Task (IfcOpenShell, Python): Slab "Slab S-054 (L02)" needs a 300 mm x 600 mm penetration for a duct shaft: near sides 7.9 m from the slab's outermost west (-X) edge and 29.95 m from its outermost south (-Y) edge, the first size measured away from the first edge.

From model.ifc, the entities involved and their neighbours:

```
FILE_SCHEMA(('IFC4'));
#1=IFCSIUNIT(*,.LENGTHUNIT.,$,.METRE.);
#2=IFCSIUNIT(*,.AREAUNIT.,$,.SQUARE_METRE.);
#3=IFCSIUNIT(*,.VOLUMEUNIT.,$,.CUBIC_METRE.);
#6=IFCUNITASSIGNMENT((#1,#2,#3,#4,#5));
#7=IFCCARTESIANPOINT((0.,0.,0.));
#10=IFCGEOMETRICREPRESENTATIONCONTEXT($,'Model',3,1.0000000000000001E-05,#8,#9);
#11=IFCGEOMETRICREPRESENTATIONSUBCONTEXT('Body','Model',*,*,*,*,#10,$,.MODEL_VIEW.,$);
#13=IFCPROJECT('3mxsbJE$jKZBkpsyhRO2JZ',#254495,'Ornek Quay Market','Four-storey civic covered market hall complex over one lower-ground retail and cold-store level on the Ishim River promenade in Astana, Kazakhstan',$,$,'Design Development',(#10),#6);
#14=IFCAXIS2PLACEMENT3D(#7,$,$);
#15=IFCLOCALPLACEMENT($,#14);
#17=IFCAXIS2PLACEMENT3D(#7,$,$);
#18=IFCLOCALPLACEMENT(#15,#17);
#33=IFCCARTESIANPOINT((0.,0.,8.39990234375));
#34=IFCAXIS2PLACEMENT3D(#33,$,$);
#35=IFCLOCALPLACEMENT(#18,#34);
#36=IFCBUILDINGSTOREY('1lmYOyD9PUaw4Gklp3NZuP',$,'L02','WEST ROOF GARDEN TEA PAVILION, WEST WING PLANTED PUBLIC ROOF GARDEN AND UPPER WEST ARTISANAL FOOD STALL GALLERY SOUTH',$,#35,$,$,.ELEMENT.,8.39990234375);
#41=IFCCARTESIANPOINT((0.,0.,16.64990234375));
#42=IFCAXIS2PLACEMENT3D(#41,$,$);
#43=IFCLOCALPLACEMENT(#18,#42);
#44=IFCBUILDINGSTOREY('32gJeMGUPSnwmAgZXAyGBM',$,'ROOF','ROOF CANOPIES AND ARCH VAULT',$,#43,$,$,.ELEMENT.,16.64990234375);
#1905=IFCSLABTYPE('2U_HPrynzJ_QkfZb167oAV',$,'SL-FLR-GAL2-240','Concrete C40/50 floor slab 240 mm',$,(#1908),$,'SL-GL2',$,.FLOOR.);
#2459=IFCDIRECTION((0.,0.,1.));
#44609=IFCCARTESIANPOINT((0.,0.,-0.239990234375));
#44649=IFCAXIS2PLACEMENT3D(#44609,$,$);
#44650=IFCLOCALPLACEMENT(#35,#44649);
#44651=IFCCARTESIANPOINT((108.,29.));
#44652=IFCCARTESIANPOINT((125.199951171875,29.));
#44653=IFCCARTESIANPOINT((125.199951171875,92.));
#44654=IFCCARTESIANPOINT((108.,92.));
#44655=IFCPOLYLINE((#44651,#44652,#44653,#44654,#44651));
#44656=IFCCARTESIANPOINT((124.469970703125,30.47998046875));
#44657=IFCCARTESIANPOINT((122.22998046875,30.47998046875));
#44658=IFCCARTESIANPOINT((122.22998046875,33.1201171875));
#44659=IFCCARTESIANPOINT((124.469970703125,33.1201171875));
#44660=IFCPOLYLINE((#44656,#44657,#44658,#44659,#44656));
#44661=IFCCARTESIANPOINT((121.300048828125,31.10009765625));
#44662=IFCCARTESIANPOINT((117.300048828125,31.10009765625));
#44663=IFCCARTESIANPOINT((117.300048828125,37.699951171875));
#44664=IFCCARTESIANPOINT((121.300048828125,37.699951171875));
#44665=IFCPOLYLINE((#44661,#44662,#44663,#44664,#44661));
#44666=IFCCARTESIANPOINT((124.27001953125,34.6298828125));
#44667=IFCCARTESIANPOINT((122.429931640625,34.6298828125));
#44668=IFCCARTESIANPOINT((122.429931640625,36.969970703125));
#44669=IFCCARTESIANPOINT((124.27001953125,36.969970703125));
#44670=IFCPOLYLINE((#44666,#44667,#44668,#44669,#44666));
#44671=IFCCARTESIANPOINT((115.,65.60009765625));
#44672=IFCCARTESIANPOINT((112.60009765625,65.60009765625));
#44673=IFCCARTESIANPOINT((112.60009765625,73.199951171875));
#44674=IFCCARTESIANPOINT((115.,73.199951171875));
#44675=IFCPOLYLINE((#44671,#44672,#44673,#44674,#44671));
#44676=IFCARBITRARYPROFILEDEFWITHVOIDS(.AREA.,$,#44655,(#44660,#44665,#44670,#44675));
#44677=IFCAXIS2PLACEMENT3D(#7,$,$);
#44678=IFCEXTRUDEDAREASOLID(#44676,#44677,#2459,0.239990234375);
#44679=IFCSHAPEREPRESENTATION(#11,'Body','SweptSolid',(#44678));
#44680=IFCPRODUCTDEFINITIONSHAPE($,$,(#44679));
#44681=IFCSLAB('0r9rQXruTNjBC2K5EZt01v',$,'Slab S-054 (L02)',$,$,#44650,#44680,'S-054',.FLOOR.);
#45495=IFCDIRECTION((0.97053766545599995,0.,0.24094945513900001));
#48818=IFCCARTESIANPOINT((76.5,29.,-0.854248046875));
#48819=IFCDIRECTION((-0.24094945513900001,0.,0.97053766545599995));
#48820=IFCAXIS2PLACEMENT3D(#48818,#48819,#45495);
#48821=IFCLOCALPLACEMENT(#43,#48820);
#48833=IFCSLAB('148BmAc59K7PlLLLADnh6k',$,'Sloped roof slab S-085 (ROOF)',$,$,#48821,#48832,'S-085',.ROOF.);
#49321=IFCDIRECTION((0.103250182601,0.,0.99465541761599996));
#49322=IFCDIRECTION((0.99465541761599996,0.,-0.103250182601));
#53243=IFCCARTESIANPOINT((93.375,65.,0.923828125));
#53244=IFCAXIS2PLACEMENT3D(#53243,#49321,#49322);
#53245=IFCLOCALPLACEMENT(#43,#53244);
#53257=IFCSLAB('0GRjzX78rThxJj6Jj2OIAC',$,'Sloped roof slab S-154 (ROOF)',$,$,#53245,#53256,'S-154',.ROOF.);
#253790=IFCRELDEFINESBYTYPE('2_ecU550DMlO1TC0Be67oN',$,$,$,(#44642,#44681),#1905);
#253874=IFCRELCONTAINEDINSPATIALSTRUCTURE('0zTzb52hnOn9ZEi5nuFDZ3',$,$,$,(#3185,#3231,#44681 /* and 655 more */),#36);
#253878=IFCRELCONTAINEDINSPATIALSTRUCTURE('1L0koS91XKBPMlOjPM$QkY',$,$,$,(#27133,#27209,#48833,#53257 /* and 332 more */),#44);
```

```python
import numpy as np
import ifcopenshell
import ifcopenshell.api.feature
import ifcopenshell.api.geometry
import ifcopenshell.api.root
import ifcopenshell.geom
import ifcopenshell.util.placement
import ifcopenshell.util.representation
import ifcopenshell.util.shape
import ifcopenshell.util.unit

model = ifcopenshell.open("model.ifc")
unit_scale = ifcopenshell.util.unit.calculate_unit_scale(model)
settings = ifcopenshell.geom.settings()


def volume(element):
    """Net volume in cubic metres, openings subtracted."""
    shape = ifcopenshell.geom.create_shape(settings, element)
    return ifcopenshell.util.shape.get_volume(shape.geometry)


slab = model.by_guid("0r9rQXruTNjBC2K5EZt01v")
before = volume(slab)

# Extent in the slab's own axes, in metres. The edges named are its -X and -Y sides.
slab_shape = ifcopenshell.geom.create_shape(settings, slab)
vertices = ifcopenshell.util.shape.get_vertices(slab_shape.geometry)
x_min, y_min, bottom = vertices.min(axis=0)
top = vertices[:, 2].max()

opening = ifcopenshell.api.root.create_entity(model, ifc_class="IfcOpeningElement", name="Duct shaft opening", predefined_type="OPENING")
context = ifcopenshell.util.representation.get_context(model, "Model", "Body", "MODEL_VIEW")
width, depth = 0.3, 0.6
outline = [(0.0, 0.0), (width, 0.0), (width, depth), (0.0, depth), (0.0, 0.0)]
# Overshoot both faces by 50 mm so the cut is clean.
shape = ifcopenshell.api.geometry.add_slab_representation(
    model, context=context, depth=top - bottom + 0.1, polyline=outline
)
ifcopenshell.api.geometry.assign_representation(model, product=opening, representation=shape)

matrix = ifcopenshell.util.placement.get_local_placement(slab.ObjectPlacement)
matrix[:, 3] = matrix @ np.append(np.array([x_min + 7.9, y_min + 29.95, bottom - 0.05]) / unit_scale, 1.0)
ifcopenshell.api.geometry.edit_object_placement(model, product=opening, matrix=matrix, is_si=False)
ifcopenshell.api.feature.add_feature(model, feature=opening, element=slab)

after = volume(slab)

print(f"slab volume {before:.3f} -> {after:.3f} m3")

model.write("model-out.ifc")
```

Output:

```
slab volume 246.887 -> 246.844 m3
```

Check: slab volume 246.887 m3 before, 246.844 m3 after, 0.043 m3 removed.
